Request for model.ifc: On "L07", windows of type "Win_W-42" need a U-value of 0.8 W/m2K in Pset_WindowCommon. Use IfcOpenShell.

First a look at what the model holds.

```python
import ifcopenshell
import ifcopenshell.util.element

model = ifcopenshell.open("model.ifc")
print(model.schema)
storey = next(s for s in model.by_type("IfcBuildingStorey") if s.Name == "L07")
windows = [e for e in ifcopenshell.util.element.get_decomposition(storey) if e.is_a("IfcWindow")]
seen = {}
for e in windows:
    element_type = ifcopenshell.util.element.get_type(e)
    key = (element_type.Name if element_type != e and element_type else None, ifcopenshell.util.element.get_pset(e, "Pset_WindowCommon", "ThermalTransmittance"))
    seen[key] = seen.get(key, 0) + 1
for (name, value), count in sorted(seen.items(), key=str):
    print(count, "x", name, "|", value)
```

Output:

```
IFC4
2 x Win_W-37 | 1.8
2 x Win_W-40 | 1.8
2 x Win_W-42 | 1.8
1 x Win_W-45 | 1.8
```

```python
import ifcopenshell
import ifcopenshell.api.pset
import ifcopenshell.util.element

model = ifcopenshell.open("model.ifc")

storey = next(s for s in model.by_type("IfcBuildingStorey") if s.Name == "L07")
windows = [e for e in ifcopenshell.util.element.get_decomposition(storey) if e.is_a("IfcWindow")]

count = 0
for e in windows:
    element_type = ifcopenshell.util.element.get_type(e)
    if element_type in (None, e) or element_type.Name != "Win_W-42":
        continue
    # add_pset returns the element's existing set when there is one.
    pset = ifcopenshell.api.pset.add_pset(model, product=e, name="Pset_WindowCommon")
    ifcopenshell.api.pset.edit_pset(model, pset=pset, properties={"ThermalTransmittance": 0.8})
    count += 1

print(count, "windows updated")

model.write("model_edited.ifc")
```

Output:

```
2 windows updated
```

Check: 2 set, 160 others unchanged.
